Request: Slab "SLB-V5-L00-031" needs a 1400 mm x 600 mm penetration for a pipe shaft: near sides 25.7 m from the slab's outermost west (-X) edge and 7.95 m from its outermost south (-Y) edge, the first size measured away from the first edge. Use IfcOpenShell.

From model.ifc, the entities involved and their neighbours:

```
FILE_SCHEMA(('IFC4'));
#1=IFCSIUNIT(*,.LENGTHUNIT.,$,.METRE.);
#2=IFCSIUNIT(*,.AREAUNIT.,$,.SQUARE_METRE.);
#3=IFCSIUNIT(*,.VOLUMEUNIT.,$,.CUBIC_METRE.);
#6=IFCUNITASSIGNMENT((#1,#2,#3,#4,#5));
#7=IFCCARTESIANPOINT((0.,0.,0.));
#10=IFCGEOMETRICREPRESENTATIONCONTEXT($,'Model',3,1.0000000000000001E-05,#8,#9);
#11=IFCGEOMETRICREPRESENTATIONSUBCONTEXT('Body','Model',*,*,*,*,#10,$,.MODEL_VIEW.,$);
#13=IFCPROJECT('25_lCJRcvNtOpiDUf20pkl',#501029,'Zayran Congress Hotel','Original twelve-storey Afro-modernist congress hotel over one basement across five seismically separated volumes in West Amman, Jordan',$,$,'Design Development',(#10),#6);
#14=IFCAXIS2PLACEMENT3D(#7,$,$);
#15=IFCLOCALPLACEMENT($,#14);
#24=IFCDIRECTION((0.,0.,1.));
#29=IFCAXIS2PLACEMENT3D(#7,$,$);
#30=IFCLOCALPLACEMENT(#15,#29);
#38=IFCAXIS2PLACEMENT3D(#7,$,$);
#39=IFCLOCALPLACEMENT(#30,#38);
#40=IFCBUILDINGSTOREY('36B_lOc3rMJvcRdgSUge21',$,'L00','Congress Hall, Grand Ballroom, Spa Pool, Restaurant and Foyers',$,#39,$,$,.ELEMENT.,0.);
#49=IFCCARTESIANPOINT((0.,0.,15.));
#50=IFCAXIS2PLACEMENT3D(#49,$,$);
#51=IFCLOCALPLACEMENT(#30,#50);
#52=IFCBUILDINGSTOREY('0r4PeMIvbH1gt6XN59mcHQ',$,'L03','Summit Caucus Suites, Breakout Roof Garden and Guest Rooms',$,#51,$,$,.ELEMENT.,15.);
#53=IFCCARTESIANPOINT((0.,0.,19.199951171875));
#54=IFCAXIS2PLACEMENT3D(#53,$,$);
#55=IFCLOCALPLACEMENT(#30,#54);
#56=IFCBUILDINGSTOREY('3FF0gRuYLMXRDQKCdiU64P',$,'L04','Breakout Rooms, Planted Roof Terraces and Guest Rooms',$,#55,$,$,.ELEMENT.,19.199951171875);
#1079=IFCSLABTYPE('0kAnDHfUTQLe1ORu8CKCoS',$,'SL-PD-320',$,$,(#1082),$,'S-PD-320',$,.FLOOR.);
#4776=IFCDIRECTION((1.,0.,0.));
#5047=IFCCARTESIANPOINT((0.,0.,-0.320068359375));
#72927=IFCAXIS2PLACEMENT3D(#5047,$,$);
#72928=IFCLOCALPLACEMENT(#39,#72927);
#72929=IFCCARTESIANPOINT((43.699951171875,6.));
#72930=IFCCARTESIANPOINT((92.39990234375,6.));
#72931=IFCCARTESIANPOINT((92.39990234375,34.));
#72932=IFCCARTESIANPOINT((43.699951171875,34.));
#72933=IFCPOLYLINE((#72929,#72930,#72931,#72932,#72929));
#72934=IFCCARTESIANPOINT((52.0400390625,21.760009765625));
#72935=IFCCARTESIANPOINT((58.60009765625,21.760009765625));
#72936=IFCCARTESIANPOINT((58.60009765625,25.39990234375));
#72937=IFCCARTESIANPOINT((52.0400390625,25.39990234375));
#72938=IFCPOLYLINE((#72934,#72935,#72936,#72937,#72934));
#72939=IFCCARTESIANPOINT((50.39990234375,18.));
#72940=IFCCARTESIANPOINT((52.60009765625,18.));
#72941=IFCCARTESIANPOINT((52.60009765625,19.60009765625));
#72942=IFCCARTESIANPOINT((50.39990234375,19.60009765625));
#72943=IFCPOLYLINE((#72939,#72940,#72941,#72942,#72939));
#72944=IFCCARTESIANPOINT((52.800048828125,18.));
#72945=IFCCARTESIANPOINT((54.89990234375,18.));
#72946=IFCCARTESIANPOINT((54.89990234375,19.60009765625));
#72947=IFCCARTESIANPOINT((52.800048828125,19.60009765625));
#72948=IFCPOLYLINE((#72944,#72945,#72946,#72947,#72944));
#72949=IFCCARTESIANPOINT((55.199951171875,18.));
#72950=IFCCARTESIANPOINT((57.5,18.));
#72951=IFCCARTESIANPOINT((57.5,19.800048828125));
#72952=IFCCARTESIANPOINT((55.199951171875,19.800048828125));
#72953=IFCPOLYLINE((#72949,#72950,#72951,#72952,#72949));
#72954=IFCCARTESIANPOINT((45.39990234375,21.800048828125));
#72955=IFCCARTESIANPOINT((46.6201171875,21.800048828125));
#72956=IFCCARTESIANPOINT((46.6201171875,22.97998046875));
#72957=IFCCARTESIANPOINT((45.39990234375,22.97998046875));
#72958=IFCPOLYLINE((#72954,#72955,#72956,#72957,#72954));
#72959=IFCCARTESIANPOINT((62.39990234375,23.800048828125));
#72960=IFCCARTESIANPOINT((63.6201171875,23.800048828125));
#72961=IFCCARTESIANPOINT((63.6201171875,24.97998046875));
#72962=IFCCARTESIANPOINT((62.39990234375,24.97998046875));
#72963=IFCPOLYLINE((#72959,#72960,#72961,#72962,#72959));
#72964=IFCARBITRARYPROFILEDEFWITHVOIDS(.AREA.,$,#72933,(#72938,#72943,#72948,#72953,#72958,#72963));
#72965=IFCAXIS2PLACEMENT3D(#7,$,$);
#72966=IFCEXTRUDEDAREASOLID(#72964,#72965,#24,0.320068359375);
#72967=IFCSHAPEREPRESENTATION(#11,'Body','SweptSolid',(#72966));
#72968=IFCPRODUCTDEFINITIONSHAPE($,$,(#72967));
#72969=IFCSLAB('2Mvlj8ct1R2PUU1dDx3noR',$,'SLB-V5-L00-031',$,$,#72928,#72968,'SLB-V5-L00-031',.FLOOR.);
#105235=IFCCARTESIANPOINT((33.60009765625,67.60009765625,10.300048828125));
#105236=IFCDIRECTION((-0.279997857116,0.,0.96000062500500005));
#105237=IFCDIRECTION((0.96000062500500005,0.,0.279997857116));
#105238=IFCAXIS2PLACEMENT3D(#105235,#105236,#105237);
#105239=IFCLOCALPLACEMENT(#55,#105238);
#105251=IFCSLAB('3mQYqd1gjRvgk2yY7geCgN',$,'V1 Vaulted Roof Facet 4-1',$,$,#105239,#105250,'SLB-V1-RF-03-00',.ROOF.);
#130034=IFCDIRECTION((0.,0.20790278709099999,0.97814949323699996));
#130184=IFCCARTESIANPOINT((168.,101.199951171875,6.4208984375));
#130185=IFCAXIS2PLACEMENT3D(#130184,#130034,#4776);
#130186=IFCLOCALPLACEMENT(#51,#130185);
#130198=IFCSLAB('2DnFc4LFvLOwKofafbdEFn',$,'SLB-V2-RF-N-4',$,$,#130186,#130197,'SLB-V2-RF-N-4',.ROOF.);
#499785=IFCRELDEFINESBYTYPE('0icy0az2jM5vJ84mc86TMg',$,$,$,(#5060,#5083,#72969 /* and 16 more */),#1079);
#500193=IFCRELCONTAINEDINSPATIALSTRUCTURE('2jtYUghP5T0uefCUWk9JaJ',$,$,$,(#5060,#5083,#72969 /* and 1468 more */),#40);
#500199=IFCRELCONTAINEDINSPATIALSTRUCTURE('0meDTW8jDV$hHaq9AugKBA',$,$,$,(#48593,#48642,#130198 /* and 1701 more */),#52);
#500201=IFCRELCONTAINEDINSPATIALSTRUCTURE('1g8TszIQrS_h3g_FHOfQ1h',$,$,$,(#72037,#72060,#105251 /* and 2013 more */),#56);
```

```python
import numpy as np
import ifcopenshell
import ifcopenshell.api.feature
import ifcopenshell.api.geometry
import ifcopenshell.api.root
import ifcopenshell.geom
import ifcopenshell.util.placement
import ifcopenshell.util.representation
import ifcopenshell.util.shape
import ifcopenshell.util.unit

model = ifcopenshell.open("model.ifc")
unit_scale = ifcopenshell.util.unit.calculate_unit_scale(model)
settings = ifcopenshell.geom.settings()


def volume(element):
    """Net volume in cubic metres, openings subtracted."""
    shape = ifcopenshell.geom.create_shape(settings, element)
    return ifcopenshell.util.shape.get_volume(shape.geometry)


slab = model.by_guid("2Mvlj8ct1R2PUU1dDx3noR")
before = volume(slab)

# Extent in the slab's own axes, in metres. The edges named are its -X and -Y sides.
slab_shape = ifcopenshell.geom.create_shape(settings, slab)
vertices = ifcopenshell.util.shape.get_vertices(slab_shape.geometry)
x_min, y_min, bottom = vertices.min(axis=0)
top = vertices[:, 2].max()

opening = ifcopenshell.api.root.create_entity(model, ifc_class="IfcOpeningElement", name="Pipe shaft opening", predefined_type="OPENING")
context = ifcopenshell.util.representation.get_context(model, "Model", "Body", "MODEL_VIEW")
width, depth = 1.4, 0.6
outline = [(0.0, 0.0), (width, 0.0), (width, depth), (0.0, depth), (0.0, 0.0)]
# Overshoot both faces by 50 mm so the cut is clean.
shape = ifcopenshell.api.geometry.add_slab_representation(
    model, context=context, depth=top - bottom + 0.1, polyline=outline
)
ifcopenshell.api.geometry.assign_representation(model, product=opening, representation=shape)

matrix = ifcopenshell.util.placement.get_local_placement(slab.ObjectPlacement)
matrix[:, 3] = matrix @ np.append(np.array([x_min + 25.7, y_min + 7.95, bottom - 0.05]) / unit_scale, 1.0)
ifcopenshell.api.geometry.edit_object_placement(model, product=opening, matrix=matrix, is_si=False)
ifcopenshell.api.feature.add_feature(model, feature=opening, element=slab)

after = volume(slab)

print(f"slab volume {before:.3f} -> {after:.3f} m3")

model.write("model_rev.ifc")
```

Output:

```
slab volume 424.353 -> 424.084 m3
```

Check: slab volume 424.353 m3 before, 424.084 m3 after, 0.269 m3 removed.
